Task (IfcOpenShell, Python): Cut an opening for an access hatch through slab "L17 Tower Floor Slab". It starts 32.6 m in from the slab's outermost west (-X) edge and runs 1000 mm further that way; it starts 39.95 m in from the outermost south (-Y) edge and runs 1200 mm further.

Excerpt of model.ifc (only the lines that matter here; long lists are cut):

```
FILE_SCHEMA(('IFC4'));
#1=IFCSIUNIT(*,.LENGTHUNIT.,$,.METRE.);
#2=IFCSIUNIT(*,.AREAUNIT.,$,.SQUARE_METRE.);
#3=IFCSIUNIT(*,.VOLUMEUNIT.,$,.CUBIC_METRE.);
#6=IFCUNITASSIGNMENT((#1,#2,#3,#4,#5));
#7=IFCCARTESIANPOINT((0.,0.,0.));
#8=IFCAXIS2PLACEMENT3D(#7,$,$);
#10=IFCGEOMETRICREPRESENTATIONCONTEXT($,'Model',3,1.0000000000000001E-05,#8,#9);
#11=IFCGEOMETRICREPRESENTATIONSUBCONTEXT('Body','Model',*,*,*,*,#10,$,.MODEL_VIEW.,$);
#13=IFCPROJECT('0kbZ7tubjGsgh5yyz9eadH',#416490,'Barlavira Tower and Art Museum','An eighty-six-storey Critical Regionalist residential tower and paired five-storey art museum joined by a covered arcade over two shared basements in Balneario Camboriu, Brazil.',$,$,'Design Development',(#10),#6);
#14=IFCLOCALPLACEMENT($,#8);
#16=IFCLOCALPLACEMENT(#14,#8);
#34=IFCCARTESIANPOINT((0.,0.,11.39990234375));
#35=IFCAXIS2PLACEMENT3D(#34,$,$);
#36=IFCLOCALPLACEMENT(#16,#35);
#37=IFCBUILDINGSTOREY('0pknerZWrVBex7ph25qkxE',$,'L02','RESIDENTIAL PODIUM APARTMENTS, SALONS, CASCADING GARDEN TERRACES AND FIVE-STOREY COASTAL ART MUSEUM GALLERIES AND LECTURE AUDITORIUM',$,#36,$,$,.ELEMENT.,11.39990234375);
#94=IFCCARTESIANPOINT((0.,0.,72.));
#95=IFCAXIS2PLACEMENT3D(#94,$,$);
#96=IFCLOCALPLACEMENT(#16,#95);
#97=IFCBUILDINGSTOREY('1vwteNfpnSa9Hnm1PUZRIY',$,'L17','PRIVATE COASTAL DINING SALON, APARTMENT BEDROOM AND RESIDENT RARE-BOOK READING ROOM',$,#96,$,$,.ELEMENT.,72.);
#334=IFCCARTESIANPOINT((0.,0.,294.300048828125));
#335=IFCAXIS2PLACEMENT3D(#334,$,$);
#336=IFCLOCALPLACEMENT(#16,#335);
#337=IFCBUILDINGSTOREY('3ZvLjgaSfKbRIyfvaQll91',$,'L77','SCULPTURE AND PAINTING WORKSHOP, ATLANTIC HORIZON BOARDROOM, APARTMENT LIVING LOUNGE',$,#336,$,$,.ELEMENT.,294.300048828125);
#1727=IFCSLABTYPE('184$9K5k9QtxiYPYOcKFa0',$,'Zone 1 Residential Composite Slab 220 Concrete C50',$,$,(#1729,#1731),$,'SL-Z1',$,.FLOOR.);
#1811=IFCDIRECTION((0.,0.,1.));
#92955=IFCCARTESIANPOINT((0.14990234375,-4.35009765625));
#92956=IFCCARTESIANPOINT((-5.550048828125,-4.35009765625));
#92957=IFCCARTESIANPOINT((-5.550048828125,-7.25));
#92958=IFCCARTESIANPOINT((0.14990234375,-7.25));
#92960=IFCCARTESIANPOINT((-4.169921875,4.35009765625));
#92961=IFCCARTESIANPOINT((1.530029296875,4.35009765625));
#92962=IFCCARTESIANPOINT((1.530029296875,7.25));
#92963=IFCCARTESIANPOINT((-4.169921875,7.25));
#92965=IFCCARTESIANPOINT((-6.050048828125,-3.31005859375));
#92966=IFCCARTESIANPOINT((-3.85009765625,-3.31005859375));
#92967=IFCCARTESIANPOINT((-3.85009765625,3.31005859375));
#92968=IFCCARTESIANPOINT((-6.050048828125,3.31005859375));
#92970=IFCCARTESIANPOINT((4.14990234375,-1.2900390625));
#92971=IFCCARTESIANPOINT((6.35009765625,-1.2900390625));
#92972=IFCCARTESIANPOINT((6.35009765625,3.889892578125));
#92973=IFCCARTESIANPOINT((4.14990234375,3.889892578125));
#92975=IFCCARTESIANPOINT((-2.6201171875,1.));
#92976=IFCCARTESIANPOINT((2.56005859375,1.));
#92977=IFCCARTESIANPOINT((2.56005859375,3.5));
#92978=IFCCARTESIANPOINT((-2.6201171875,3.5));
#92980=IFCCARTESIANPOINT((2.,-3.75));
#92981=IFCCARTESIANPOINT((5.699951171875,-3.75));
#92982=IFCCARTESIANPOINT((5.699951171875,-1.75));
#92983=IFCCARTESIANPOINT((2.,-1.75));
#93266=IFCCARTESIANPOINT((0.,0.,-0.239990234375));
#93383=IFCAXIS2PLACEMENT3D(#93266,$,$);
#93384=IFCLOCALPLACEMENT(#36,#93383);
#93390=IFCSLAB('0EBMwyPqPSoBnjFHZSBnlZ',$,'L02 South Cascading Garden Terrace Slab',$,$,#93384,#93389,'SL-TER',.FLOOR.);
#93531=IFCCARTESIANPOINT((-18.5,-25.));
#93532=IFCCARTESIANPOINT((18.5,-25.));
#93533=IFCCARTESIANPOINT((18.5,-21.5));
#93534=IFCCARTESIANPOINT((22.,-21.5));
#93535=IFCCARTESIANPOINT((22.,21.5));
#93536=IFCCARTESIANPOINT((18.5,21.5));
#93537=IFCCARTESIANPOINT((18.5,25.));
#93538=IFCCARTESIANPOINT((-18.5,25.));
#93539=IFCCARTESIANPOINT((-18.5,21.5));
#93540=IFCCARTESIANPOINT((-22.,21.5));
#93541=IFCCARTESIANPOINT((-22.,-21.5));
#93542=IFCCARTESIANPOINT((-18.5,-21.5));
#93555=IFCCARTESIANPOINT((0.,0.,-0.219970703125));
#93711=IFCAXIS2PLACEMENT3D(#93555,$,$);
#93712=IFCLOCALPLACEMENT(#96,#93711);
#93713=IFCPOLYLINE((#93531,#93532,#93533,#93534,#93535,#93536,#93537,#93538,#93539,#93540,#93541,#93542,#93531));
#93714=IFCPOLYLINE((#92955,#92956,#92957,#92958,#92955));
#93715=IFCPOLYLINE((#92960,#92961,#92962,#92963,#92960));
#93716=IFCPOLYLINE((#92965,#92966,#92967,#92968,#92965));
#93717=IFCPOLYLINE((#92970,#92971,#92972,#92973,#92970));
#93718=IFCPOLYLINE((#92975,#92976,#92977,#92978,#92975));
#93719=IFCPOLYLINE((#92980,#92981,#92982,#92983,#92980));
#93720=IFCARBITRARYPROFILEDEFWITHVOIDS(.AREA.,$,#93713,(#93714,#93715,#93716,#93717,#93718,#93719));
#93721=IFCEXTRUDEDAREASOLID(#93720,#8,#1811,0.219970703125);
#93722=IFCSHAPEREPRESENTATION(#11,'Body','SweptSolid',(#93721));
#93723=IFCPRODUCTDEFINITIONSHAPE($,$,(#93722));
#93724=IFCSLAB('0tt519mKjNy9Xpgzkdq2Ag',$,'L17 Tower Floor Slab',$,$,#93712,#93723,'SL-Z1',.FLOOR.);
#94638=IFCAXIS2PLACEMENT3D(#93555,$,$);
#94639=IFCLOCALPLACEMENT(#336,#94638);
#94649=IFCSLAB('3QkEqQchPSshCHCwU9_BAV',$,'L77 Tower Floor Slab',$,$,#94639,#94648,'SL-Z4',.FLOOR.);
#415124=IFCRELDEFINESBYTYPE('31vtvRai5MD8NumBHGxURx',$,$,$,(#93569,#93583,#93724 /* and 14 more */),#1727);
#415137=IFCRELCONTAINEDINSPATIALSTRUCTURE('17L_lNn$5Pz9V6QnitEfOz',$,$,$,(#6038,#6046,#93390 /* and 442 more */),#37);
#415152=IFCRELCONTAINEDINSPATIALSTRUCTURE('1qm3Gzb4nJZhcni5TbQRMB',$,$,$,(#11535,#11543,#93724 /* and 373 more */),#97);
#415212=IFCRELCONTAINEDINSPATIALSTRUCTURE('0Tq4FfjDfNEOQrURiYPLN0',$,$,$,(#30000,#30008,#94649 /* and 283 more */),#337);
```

```python
import numpy as np
import ifcopenshell
import ifcopenshell.api.feature
import ifcopenshell.api.geometry
import ifcopenshell.api.root
import ifcopenshell.geom
import ifcopenshell.util.placement
import ifcopenshell.util.representation
import ifcopenshell.util.shape
import ifcopenshell.util.unit

model = ifcopenshell.open("model.ifc")
unit_scale = ifcopenshell.util.unit.calculate_unit_scale(model)
settings = ifcopenshell.geom.settings()


def volume(element):
    """Net volume in cubic metres, openings subtracted."""
    shape = ifcopenshell.geom.create_shape(settings, element)
    return ifcopenshell.util.shape.get_volume(shape.geometry)


slab = model.by_guid("0tt519mKjNy9Xpgzkdq2Ag")
before = volume(slab)

# Extent in the slab's own axes, in metres. The edges named are its -X and -Y sides.
slab_shape = ifcopenshell.geom.create_shape(settings, slab)
vertices = ifcopenshell.util.shape.get_vertices(slab_shape.geometry)
x_min, y_min, bottom = vertices.min(axis=0)
top = vertices[:, 2].max()

opening = ifcopenshell.api.root.create_entity(model, ifc_class="IfcOpeningElement", name="Access hatch opening", predefined_type="OPENING")
context = ifcopenshell.util.representation.get_context(model, "Model", "Body", "MODEL_VIEW")
width, depth = 1, 1.2
outline = [(0.0, 0.0), (width, 0.0), (width, depth), (0.0, depth), (0.0, 0.0)]
# Overshoot both faces by 50 mm so the cut is clean.
shape = ifcopenshell.api.geometry.add_slab_representation(
    model, context=context, depth=top - bottom + 0.1, polyline=outline
)
ifcopenshell.api.geometry.assign_representation(model, product=opening, representation=shape)

matrix = ifcopenshell.util.placement.get_local_placement(slab.ObjectPlacement)
matrix[:, 3] = matrix @ np.append(np.array([x_min + 32.6, y_min + 39.95, bottom - 0.05]) / unit_scale, 1.0)
ifcopenshell.api.geometry.edit_object_placement(model, product=opening, matrix=matrix, is_si=False)
ifcopenshell.api.feature.add_feature(model, feature=opening, element=slab)

after = volume(slab)

print(f"slab volume {before:.3f} -> {after:.3f} m3")

model.write("model_updated.ifc")
```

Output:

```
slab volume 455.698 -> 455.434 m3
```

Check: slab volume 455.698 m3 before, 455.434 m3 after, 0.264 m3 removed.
